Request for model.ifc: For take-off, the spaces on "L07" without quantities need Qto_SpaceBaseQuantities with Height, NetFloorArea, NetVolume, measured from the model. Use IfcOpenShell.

First a look at what the model holds.

```python
import ifcopenshell
import ifcopenshell.util.element
import ifcopenshell.util.unit

model = ifcopenshell.open("model.ifc")
print(model.schema)
for unit_type in ("LENGTHUNIT", "AREAUNIT", "VOLUMEUNIT"):
    print(unit_type, ifcopenshell.util.unit.calculate_unit_scale(model, unit_type))
storey = next(s for s in model.by_type("IfcBuildingStorey") if s.Name == "L07")
spaces = [e for e in ifcopenshell.util.element.get_decomposition(storey) if e.is_a("IfcSpace")]
for e in sorted(spaces, key=lambda e: e.id()):
    print(e.id(), e.is_a(), e.Name, list(ifcopenshell.util.element.get_psets(e, qtos_only=True)), sep=" | ")
```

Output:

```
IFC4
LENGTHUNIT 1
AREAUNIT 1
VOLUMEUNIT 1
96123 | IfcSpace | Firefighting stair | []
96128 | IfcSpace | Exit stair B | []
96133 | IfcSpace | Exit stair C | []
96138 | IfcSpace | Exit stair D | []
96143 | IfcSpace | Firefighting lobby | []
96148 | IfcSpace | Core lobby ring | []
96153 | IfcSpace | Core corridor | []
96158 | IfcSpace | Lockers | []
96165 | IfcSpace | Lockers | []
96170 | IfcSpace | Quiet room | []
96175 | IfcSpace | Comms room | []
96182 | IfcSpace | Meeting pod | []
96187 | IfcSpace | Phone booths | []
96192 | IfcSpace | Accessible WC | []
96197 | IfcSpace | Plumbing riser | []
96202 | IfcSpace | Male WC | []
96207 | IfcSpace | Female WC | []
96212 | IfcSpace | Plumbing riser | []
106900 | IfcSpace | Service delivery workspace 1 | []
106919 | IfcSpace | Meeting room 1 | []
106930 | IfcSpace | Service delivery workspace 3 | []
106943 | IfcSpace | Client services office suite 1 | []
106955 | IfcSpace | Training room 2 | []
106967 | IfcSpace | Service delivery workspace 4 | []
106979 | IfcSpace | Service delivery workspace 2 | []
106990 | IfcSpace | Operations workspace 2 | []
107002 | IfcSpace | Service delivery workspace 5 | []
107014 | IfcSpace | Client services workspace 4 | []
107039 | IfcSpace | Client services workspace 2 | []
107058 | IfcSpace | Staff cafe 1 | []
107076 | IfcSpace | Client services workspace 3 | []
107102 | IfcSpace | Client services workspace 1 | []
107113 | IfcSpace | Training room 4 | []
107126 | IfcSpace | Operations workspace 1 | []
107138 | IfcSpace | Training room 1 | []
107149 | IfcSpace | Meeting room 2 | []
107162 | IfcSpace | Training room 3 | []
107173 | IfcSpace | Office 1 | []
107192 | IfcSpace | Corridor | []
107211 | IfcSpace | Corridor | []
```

```python
import ifcopenshell
import ifcopenshell.api.pset
import ifcopenshell.geom
import ifcopenshell.util.element
import ifcopenshell.util.shape
import ifcopenshell.util.unit

model = ifcopenshell.open("model.ifc")
unit_scale = ifcopenshell.util.unit.calculate_unit_scale(model)
area_scale = ifcopenshell.util.unit.calculate_unit_scale(model, "AREAUNIT")
volume_scale = ifcopenshell.util.unit.calculate_unit_scale(model, "VOLUMEUNIT")
settings = ifcopenshell.geom.settings()

storey = next(s for s in model.by_type("IfcBuildingStorey") if s.Name == "L07")
spaces = [e for e in ifcopenshell.util.element.get_decomposition(storey) if e.is_a("IfcSpace")]

for e in sorted(spaces, key=lambda e: e.id()):
    if ifcopenshell.util.element.get_psets(e, qtos_only=True, should_inherit=False):
        continue
    # Geometry comes back in metres, in the element's own axes.
    shape = ifcopenshell.geom.create_shape(settings, e)
    values = {
        "Height": ifcopenshell.util.shape.get_z(shape.geometry) / unit_scale,
        "NetFloorArea": ifcopenshell.util.shape.get_footprint_area(shape.geometry) / area_scale,
        "NetVolume": ifcopenshell.util.shape.get_volume(shape.geometry) / volume_scale,
    }
    qto = ifcopenshell.api.pset.add_qto(model, product=e, name="Qto_SpaceBaseQuantities")
    ifcopenshell.api.pset.edit_qto(model, qto=qto, properties=values)
    print(e.id(), {k: round(v, 3) for k, v in values.items()})

model.write("model-out.ifc")
```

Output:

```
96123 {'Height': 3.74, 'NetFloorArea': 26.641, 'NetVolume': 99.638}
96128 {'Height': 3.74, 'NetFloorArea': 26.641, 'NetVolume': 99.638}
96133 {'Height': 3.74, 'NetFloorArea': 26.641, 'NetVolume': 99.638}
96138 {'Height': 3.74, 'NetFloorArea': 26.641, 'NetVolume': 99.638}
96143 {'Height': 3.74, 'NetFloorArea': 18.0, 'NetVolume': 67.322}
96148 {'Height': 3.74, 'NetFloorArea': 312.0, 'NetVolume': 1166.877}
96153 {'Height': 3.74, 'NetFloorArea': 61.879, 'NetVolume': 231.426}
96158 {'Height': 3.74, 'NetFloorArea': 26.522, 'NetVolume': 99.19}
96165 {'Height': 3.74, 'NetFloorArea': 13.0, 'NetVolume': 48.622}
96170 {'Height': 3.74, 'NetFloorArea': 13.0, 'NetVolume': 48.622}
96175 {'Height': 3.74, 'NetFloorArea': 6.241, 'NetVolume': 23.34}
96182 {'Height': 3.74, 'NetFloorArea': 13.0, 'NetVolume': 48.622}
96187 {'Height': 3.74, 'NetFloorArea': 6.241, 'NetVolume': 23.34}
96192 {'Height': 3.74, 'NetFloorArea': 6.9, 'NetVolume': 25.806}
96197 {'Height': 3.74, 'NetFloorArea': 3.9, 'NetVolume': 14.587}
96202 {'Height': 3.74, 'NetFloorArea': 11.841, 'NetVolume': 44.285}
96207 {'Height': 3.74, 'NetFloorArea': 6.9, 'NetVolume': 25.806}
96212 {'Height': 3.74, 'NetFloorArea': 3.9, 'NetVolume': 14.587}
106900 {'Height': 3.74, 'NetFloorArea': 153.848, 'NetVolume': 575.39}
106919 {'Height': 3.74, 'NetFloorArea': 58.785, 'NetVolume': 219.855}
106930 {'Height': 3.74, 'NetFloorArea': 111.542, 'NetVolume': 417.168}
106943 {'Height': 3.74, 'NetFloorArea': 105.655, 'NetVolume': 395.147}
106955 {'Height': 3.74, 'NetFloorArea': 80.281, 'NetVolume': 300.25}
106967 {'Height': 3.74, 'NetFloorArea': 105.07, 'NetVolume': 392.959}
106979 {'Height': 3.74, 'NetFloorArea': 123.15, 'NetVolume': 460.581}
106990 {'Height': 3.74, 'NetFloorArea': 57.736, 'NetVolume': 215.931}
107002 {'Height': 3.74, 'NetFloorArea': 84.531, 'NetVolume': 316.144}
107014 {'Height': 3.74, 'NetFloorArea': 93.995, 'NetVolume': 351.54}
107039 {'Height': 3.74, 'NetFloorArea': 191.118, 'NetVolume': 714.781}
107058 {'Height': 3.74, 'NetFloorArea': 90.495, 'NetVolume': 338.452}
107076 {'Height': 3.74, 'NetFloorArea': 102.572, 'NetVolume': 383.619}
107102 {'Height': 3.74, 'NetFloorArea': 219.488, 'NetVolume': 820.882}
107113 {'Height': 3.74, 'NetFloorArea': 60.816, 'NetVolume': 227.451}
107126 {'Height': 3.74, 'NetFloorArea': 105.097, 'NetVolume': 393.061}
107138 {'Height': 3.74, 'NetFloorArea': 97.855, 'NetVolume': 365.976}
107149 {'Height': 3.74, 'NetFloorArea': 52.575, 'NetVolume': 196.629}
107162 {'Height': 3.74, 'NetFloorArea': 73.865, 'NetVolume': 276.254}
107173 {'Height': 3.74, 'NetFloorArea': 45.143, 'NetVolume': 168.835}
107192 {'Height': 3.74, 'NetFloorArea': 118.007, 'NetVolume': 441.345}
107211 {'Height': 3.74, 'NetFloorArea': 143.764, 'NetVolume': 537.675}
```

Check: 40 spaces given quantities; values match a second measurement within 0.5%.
